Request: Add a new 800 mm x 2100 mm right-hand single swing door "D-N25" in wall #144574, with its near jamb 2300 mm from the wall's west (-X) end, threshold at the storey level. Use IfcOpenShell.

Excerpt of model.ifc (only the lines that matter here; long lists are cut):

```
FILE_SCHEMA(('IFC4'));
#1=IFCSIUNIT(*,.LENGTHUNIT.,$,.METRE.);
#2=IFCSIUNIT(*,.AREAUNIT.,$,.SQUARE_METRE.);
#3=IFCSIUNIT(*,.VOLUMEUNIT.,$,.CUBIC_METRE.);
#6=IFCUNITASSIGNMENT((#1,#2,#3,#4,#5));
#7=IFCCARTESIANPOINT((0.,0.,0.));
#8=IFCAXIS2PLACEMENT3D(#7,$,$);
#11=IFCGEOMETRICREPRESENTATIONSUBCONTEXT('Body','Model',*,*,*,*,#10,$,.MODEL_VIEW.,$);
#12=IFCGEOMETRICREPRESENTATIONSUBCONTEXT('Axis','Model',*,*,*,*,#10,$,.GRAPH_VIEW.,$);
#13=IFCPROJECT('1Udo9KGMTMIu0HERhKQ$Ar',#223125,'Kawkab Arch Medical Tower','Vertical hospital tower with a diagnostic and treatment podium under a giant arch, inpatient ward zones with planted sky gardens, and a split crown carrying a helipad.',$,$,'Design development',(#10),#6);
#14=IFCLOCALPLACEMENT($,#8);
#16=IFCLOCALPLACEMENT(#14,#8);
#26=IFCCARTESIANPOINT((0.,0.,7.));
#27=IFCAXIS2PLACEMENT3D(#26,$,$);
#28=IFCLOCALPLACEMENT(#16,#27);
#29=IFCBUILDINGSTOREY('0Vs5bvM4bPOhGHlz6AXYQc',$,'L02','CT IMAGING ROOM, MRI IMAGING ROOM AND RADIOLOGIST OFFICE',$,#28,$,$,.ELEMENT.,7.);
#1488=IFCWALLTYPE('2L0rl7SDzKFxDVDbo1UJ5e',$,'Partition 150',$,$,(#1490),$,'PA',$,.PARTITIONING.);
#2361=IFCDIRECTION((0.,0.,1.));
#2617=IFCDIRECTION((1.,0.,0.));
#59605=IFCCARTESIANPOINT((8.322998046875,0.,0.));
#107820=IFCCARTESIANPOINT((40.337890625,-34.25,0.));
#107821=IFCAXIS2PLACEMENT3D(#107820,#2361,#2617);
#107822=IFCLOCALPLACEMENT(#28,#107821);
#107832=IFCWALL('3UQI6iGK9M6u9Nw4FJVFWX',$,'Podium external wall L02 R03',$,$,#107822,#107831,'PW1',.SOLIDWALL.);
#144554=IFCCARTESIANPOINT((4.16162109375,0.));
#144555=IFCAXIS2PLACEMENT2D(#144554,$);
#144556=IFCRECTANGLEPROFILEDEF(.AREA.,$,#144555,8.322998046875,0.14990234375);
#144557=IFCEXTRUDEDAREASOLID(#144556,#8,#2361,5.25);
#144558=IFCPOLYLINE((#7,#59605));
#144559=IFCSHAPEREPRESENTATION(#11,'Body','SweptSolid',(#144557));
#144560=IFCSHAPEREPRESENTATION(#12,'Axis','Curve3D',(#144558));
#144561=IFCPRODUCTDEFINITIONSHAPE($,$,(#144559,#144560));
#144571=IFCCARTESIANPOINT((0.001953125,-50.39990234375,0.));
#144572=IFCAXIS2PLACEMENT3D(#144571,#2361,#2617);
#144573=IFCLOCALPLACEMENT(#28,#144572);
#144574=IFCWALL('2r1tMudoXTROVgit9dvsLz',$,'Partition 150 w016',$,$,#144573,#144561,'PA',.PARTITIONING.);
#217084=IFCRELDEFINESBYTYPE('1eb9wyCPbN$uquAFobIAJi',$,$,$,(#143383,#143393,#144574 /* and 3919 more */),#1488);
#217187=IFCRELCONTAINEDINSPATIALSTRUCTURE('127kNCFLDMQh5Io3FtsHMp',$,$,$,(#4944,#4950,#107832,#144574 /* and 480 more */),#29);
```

```python
import numpy as np
import ifcopenshell
import ifcopenshell.api.feature
import ifcopenshell.api.geometry
import ifcopenshell.api.root
import ifcopenshell.api.spatial
import ifcopenshell.geom
import ifcopenshell.util.element
import ifcopenshell.util.placement
import ifcopenshell.util.representation
import ifcopenshell.util.shape
import ifcopenshell.util.unit

model = ifcopenshell.open("model.ifc")
unit_scale = ifcopenshell.util.unit.calculate_unit_scale(model)
settings = ifcopenshell.geom.settings()


def volume(element):
    """Net volume in cubic metres, openings subtracted."""
    shape = ifcopenshell.geom.create_shape(settings, element)
    return ifcopenshell.util.shape.get_volume(shape.geometry)


wall = model.by_guid("2r1tMudoXTROVgit9dvsLz")
storey = ifcopenshell.util.element.get_container(wall, ifc_class="IfcBuildingStorey")
context = ifcopenshell.util.representation.get_context(model, "Model", "Body", "MODEL_VIEW")
before = volume(wall)

width, height, from_end, sill = 0.8, 2.1, 2.3, 0.0  # metres

# The wall runs along its own X axis, and the end named is its -X end.
wall_shape = ifcopenshell.geom.create_shape(settings, wall)
x, y, z = ifcopenshell.util.shape.get_vertices(wall_shape.geometry).T
start = x.min() + from_end
face, thickness = float(y.min()), float(y.max() - y.min())
wall_matrix = ifcopenshell.util.placement.get_local_placement(wall.ObjectPlacement)
level = ifcopenshell.util.placement.get_local_placement(storey.ObjectPlacement)[2, 3]


def in_wall(x, y):
    """Placement at x, y metres in the wall's axes, at sill height."""
    matrix = wall_matrix.copy()
    matrix[:, 3] = wall_matrix @ np.array([x / unit_scale, y / unit_scale, 0.0, 1.0])
    matrix[2, 3] = level + sill / unit_scale
    return matrix


# Opening: a box that overshoots both wall faces by 50 mm.
opening = ifcopenshell.api.root.create_entity(model, ifc_class="IfcOpeningElement", predefined_type="OPENING")
box = ifcopenshell.api.geometry.add_wall_representation(
    model, context=context, length=width, height=height, thickness=thickness + 0.1
)
ifcopenshell.api.geometry.assign_representation(model, product=opening, representation=box)
ifcopenshell.api.geometry.edit_object_placement(model, product=opening, matrix=in_wall(start, face - 0.05), is_si=False)
ifcopenshell.api.feature.add_feature(model, feature=opening, element=wall)

door = ifcopenshell.api.root.create_entity(model, ifc_class="IfcDoor", name="D-N25", predefined_type="DOOR")
door.OverallWidth, door.OverallHeight = width / unit_scale, height / unit_scale
door.OperationType = "SINGLE_SWING_RIGHT"
body = ifcopenshell.api.geometry.add_door_representation(
    model,
    context=context,
    overall_width=door.OverallWidth,
    overall_height=door.OverallHeight,
    operation_type="SINGLE_SWING_RIGHT",
    lining_properties={"LiningDepth": thickness / unit_scale, "ThresholdDepth": thickness / unit_scale},
)
ifcopenshell.api.geometry.assign_representation(model, product=door, representation=body)
ifcopenshell.api.spatial.assign_container(model, products=[door], relating_structure=storey)
ifcopenshell.api.feature.add_filling(model, opening=opening, element=door)

# The lining spans the wall, so the door starts at the wall face.
ifcopenshell.api.geometry.edit_object_placement(model, product=door, matrix=in_wall(start, face), is_si=False)

after = volume(wall)

print(f"wall volume {before:.3f} -> {after:.3f} m3")

model.write("model_v2.ifc")
```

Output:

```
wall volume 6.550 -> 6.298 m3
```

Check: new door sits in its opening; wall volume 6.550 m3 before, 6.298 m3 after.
